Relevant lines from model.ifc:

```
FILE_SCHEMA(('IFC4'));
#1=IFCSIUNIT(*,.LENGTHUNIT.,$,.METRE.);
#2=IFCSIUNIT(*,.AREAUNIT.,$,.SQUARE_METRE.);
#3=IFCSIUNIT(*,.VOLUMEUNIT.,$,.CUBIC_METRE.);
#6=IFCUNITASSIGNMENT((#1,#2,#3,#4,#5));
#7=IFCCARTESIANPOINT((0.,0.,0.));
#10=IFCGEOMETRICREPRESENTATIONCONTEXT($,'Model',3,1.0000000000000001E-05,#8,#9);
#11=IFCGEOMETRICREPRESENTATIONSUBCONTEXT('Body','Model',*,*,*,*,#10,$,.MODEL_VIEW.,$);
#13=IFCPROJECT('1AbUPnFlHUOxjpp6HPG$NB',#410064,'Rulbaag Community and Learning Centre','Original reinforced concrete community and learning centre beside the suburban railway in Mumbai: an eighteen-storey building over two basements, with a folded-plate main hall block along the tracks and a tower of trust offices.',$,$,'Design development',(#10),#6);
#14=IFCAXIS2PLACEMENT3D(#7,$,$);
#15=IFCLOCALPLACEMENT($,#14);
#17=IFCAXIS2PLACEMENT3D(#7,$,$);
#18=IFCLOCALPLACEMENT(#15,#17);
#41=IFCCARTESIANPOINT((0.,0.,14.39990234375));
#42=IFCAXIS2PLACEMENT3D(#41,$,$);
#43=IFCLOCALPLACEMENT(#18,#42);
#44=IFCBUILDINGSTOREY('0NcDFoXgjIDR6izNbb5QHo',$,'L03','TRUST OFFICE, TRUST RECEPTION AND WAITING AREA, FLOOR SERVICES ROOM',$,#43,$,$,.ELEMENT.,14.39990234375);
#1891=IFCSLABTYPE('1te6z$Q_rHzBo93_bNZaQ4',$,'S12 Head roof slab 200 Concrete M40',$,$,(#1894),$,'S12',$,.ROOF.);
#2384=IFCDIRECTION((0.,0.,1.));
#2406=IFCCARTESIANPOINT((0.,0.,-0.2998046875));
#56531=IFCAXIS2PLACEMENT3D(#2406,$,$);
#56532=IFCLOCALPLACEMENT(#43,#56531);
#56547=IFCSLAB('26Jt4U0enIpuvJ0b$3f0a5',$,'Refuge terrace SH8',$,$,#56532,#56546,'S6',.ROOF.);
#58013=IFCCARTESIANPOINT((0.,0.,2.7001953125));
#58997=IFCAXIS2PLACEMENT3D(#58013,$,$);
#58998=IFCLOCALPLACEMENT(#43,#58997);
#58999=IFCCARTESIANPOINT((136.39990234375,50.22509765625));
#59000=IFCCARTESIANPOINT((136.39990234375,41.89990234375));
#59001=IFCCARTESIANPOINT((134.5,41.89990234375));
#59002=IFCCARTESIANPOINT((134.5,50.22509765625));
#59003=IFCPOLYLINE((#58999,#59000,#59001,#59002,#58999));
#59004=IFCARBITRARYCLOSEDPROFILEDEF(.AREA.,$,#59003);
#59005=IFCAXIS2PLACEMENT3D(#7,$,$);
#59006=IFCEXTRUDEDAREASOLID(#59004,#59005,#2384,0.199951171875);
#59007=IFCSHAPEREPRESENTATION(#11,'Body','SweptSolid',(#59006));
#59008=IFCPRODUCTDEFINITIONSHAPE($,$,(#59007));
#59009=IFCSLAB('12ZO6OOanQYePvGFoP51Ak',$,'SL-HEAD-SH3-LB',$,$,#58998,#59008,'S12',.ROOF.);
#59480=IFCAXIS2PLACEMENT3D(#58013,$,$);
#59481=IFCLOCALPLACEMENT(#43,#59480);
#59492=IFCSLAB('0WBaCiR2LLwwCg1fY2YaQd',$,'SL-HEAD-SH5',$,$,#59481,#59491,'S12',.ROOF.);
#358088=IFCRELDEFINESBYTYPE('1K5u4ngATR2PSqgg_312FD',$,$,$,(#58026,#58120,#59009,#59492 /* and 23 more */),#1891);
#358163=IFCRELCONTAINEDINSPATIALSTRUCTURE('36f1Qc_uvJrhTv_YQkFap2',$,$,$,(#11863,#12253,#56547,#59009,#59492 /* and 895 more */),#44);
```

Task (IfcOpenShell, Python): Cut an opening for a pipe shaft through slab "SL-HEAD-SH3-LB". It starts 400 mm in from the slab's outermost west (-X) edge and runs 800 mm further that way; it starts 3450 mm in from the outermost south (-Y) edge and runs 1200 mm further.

```python
import numpy as np
import ifcopenshell
import ifcopenshell.api.feature
import ifcopenshell.api.geometry
import ifcopenshell.api.root
import ifcopenshell.geom
import ifcopenshell.util.placement
import ifcopenshell.util.representation
import ifcopenshell.util.shape
import ifcopenshell.util.unit

model = ifcopenshell.open("model.ifc")
unit_scale = ifcopenshell.util.unit.calculate_unit_scale(model)
settings = ifcopenshell.geom.settings()


def volume(element):
    """Net volume in cubic metres, openings subtracted."""
    shape = ifcopenshell.geom.create_shape(settings, element)
    return ifcopenshell.util.shape.get_volume(shape.geometry)


slab = model.by_guid("12ZO6OOanQYePvGFoP51Ak")
before = volume(slab)

# Extent in the slab's own axes, in metres. The edges named are its -X and -Y sides.
slab_shape = ifcopenshell.geom.create_shape(settings, slab)
vertices = ifcopenshell.util.shape.get_vertices(slab_shape.geometry)
x_min, y_min, bottom = vertices.min(axis=0)
top = vertices[:, 2].max()

opening = ifcopenshell.api.root.create_entity(model, ifc_class="IfcOpeningElement", name="Pipe shaft opening", predefined_type="OPENING")
context = ifcopenshell.util.representation.get_context(model, "Model", "Body", "MODEL_VIEW")
width, depth = 0.8, 1.2
outline = [(0.0, 0.0), (width, 0.0), (width, depth), (0.0, depth), (0.0, 0.0)]
# Overshoot both faces by 50 mm so the cut is clean.
shape = ifcopenshell.api.geometry.add_slab_representation(
    model, context=context, depth=top - bottom + 0.1, polyline=outline
)
ifcopenshell.api.geometry.assign_representation(model, product=opening, representation=shape)

matrix = ifcopenshell.util.placement.get_local_placement(slab.ObjectPlacement)
matrix[:, 3] = matrix @ np.append(np.array([x_min + 0.4, y_min + 3.45, bottom - 0.05]) / unit_scale, 1.0)
ifcopenshell.api.geometry.edit_object_placement(model, product=opening, matrix=matrix, is_si=False)
ifcopenshell.api.feature.add_feature(model, feature=opening, element=slab)

after = volume(slab)

print(f"slab volume {before:.3f} -> {after:.3f} m3")

model.write("model_v2.ifc")
```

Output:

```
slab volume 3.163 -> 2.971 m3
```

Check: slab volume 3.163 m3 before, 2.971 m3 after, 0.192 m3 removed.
